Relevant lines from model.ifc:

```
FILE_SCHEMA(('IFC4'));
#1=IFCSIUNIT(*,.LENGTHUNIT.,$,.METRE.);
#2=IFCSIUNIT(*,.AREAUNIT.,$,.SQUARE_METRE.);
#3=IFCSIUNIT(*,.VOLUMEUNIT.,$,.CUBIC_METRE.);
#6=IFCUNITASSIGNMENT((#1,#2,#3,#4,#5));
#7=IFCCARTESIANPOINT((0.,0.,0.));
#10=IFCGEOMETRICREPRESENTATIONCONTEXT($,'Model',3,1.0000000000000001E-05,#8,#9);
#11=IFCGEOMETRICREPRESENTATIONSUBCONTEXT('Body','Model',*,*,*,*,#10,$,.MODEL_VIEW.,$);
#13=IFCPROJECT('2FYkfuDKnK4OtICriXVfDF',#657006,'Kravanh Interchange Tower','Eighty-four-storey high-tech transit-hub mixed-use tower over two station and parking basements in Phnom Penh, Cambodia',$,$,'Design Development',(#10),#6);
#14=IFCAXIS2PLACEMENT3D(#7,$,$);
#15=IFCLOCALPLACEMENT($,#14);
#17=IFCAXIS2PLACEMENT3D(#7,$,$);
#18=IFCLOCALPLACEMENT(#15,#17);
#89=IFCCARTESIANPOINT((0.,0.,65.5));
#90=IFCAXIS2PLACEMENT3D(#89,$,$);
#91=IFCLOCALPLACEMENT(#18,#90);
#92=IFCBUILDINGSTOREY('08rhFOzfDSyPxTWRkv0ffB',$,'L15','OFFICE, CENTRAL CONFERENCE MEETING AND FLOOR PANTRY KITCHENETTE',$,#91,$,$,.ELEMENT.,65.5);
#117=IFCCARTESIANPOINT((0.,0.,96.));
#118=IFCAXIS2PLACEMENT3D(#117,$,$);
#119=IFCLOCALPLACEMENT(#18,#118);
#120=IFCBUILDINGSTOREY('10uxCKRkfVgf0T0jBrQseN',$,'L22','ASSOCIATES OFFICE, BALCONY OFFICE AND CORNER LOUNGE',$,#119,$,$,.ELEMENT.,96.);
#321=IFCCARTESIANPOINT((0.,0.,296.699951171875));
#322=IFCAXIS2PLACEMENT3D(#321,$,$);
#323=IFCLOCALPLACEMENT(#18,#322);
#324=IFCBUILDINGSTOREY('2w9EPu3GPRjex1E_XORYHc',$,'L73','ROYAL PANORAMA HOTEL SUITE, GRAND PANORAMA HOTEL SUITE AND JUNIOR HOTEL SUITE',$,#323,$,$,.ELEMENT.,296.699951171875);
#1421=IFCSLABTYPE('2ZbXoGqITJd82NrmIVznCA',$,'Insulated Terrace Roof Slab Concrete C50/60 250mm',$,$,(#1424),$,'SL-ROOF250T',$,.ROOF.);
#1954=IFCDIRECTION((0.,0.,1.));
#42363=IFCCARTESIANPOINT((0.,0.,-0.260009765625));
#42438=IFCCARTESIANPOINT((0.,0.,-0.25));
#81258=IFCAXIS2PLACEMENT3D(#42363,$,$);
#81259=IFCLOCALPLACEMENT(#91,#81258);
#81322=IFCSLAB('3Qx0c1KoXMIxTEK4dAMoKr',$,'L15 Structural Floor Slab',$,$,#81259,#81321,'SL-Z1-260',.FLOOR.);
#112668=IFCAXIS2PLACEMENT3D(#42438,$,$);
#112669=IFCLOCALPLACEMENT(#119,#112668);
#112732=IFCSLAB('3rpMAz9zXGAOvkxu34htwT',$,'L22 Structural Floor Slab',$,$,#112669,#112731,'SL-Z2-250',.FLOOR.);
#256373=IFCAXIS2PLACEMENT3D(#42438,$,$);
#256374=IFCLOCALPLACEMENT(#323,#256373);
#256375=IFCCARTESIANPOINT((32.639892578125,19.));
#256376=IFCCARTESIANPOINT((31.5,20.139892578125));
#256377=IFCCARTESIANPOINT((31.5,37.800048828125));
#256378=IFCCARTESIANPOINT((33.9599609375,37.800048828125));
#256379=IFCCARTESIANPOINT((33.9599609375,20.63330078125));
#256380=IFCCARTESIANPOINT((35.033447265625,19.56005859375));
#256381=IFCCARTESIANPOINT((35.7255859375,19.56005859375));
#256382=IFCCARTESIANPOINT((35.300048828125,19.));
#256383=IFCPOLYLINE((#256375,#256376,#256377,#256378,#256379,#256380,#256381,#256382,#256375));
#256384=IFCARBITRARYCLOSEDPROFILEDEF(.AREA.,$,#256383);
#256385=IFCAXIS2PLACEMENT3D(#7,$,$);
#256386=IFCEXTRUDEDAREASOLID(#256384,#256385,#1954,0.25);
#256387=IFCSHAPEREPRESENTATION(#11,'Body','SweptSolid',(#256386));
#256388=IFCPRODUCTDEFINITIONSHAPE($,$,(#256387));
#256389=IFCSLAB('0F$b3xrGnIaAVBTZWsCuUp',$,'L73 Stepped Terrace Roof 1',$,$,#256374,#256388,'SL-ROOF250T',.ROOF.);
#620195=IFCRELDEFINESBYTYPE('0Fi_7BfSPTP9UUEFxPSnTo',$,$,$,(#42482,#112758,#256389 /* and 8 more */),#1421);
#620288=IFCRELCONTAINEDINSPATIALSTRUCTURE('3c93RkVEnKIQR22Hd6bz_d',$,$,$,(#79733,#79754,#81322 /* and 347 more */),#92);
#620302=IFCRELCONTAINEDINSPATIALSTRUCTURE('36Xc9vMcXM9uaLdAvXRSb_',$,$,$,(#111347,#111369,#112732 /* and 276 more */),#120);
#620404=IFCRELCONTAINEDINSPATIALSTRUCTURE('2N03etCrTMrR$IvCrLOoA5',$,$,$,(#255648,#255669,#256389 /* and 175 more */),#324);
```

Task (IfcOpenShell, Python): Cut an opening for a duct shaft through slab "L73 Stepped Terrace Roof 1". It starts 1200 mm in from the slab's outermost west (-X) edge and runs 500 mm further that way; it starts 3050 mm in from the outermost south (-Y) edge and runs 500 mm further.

```python
import numpy as np
import ifcopenshell
import ifcopenshell.api.feature
import ifcopenshell.api.geometry
import ifcopenshell.api.root
import ifcopenshell.geom
import ifcopenshell.util.placement
import ifcopenshell.util.representation
import ifcopenshell.util.shape
import ifcopenshell.util.unit

model = ifcopenshell.open("model.ifc")
unit_scale = ifcopenshell.util.unit.calculate_unit_scale(model)
settings = ifcopenshell.geom.settings()


def volume(element):
    """Net volume in cubic metres, openings subtracted."""
    shape = ifcopenshell.geom.create_shape(settings, element)
    return ifcopenshell.util.shape.get_volume(shape.geometry)


slab = model.by_guid("0F$b3xrGnIaAVBTZWsCuUp")
before = volume(slab)

# Extent in the slab's own axes, in metres. The edges named are its -X and -Y sides.
slab_shape = ifcopenshell.geom.create_shape(settings, slab)
vertices = ifcopenshell.util.shape.get_vertices(slab_shape.geometry)
x_min, y_min, bottom = vertices.min(axis=0)
top = vertices[:, 2].max()

opening = ifcopenshell.api.root.create_entity(model, ifc_class="IfcOpeningElement", name="Duct shaft opening", predefined_type="OPENING")
context = ifcopenshell.util.representation.get_context(model, "Model", "Body", "MODEL_VIEW")
width, depth = 0.5, 0.5
outline = [(0.0, 0.0), (width, 0.0), (width, depth), (0.0, depth), (0.0, 0.0)]
# Overshoot both faces by 50 mm so the cut is clean.
shape = ifcopenshell.api.geometry.add_slab_representation(
    model, context=context, depth=top - bottom + 0.1, polyline=outline
)
ifcopenshell.api.geometry.assign_representation(model, product=opening, representation=shape)

matrix = ifcopenshell.util.placement.get_local_placement(slab.ObjectPlacement)
matrix[:, 3] = matrix @ np.append(np.array([x_min + 1.2, y_min + 3.05, bottom - 0.05]) / unit_scale, 1.0)
ifcopenshell.api.geometry.edit_object_placement(model, product=opening, matrix=matrix, is_si=False)
ifcopenshell.api.feature.add_feature(model, feature=opening, element=slab)

after = volume(slab)

print(f"slab volume {before:.3f} -> {after:.3f} m3")

model.write("model_v2.ifc")
```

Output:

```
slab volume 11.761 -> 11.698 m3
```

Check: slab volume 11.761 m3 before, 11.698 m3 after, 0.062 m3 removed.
